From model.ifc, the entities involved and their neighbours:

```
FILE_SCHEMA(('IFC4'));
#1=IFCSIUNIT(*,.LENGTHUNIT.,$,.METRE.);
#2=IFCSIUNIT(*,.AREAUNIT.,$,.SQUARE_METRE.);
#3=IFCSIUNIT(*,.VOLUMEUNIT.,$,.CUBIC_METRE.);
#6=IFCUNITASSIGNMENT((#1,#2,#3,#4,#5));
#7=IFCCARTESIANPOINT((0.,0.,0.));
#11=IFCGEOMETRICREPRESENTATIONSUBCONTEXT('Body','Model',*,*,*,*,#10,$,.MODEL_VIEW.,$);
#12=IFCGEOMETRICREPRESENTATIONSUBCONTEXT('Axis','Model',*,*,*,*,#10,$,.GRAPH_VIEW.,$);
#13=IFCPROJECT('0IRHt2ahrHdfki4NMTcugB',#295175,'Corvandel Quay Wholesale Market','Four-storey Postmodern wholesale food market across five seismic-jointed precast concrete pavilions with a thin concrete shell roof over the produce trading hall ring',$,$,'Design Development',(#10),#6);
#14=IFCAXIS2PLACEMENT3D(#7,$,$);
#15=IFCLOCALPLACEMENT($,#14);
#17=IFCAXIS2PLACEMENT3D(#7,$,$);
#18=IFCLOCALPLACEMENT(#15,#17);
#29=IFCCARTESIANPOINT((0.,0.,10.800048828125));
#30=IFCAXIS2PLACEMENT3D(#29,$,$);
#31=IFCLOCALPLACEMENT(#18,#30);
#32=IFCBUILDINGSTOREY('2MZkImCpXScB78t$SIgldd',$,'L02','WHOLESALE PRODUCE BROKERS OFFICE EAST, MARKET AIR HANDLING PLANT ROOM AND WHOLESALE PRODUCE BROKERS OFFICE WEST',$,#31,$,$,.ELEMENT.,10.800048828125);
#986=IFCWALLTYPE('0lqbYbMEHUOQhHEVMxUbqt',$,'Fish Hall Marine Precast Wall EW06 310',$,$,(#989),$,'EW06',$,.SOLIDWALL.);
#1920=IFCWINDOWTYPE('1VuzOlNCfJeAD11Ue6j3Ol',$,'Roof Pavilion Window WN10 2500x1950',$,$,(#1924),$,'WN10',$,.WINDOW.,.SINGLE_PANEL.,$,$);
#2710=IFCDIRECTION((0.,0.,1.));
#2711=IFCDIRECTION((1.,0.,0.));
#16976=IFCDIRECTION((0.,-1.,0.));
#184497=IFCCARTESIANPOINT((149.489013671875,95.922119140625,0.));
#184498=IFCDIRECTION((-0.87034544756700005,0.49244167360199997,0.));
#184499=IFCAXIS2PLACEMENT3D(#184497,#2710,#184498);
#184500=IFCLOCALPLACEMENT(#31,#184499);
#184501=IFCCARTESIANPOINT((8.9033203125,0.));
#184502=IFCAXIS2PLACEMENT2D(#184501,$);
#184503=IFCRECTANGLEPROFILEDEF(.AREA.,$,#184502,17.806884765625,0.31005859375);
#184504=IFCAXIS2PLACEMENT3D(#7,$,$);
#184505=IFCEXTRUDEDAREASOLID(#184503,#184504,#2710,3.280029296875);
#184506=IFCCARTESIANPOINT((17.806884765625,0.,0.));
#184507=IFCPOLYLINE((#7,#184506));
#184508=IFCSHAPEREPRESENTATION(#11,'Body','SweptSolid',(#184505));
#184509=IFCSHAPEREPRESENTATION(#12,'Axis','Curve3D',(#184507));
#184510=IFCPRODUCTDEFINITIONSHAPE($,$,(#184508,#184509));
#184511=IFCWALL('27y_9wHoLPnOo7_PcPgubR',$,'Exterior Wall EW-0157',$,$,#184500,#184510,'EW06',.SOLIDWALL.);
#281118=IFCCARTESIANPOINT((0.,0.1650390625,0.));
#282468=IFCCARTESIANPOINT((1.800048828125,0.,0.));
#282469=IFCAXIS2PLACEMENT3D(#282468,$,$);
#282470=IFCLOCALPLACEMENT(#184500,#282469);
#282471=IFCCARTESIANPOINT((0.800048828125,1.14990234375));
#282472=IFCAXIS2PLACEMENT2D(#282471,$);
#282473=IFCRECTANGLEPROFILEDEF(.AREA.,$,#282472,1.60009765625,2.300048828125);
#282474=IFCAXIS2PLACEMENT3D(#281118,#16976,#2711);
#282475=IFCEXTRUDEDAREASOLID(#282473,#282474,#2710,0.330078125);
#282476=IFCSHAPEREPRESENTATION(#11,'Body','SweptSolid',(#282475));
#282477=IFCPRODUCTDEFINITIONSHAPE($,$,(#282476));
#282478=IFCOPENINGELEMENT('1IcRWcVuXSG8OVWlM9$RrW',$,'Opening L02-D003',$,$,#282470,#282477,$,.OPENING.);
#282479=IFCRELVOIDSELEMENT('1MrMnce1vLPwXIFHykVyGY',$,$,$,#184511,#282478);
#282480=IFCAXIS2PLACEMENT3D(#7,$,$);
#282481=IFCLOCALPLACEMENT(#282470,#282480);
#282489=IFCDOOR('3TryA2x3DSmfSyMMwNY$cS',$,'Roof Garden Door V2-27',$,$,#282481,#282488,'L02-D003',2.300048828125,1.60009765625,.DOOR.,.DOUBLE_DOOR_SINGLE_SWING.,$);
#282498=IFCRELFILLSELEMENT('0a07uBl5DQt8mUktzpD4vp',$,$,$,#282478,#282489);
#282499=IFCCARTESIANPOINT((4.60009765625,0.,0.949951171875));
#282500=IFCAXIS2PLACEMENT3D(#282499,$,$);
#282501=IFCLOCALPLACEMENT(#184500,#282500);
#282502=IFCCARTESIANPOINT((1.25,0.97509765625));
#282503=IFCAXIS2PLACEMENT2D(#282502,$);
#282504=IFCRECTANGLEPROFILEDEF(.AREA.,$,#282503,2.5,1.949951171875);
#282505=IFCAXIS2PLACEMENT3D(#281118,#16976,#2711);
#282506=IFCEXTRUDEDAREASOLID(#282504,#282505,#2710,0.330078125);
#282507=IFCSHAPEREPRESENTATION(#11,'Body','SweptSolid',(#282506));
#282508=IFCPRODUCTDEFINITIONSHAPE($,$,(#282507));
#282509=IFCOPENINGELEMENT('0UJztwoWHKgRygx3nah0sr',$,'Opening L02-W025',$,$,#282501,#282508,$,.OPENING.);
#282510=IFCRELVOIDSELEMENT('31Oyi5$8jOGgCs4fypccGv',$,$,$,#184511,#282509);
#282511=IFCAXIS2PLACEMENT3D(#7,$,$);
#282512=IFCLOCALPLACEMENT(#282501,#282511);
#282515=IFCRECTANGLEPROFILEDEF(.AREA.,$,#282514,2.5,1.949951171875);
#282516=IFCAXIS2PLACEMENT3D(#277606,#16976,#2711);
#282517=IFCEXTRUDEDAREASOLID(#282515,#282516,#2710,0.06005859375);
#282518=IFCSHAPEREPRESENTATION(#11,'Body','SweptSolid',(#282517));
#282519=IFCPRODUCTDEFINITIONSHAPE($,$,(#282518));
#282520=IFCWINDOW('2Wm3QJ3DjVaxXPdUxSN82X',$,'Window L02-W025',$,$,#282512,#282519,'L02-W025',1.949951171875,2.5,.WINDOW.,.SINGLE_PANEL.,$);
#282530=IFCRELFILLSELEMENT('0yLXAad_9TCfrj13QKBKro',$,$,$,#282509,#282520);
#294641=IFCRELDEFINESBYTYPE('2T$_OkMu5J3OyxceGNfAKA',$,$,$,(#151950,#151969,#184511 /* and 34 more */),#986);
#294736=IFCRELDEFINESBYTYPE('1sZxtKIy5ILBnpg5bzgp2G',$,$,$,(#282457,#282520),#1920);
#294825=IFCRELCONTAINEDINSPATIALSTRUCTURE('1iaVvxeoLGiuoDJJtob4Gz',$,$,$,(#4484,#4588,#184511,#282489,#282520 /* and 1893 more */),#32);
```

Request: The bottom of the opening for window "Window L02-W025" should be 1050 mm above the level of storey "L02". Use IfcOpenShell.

```python
import numpy as np
import ifcopenshell
import ifcopenshell.api.geometry
import ifcopenshell.geom
import ifcopenshell.util.element
import ifcopenshell.util.placement
import ifcopenshell.util.shape
import ifcopenshell.util.unit

model = ifcopenshell.open("model.ifc")
unit_scale = ifcopenshell.util.unit.calculate_unit_scale(model)

window = model.by_guid("2Wm3QJ3DjVaxXPdUxSN82X")
opening = window.FillsVoids[0].RelatingOpeningElement
storey = ifcopenshell.util.element.get_container(window, ifc_class="IfcBuildingStorey")
level = ifcopenshell.util.placement.get_local_placement(storey.ObjectPlacement)[2, 3]

# The opening's origin need not be at the sill, so measure its lowest point.
shape = ifcopenshell.geom.create_shape(ifcopenshell.geom.settings(), opening)
bottom = ifcopenshell.util.shape.get_shape_bottom_elevation(shape, shape.geometry) / unit_scale
dz = level + 1.05 / unit_scale - bottom

shift = np.array([0.0, 0.0, dz])
# The window is placed relative to its opening, so it follows when the opening moves.
matrix = ifcopenshell.util.placement.get_local_placement(opening.ObjectPlacement)
matrix[:3, 3] += shift
ifcopenshell.api.geometry.edit_object_placement(
    model, product=opening, matrix=matrix, is_si=False, should_transform_children=True
)

print(f"moved by {dz * unit_scale:+.3f} m")

model.write("model_v2.ifc")
```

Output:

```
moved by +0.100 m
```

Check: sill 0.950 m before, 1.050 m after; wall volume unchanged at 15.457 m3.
